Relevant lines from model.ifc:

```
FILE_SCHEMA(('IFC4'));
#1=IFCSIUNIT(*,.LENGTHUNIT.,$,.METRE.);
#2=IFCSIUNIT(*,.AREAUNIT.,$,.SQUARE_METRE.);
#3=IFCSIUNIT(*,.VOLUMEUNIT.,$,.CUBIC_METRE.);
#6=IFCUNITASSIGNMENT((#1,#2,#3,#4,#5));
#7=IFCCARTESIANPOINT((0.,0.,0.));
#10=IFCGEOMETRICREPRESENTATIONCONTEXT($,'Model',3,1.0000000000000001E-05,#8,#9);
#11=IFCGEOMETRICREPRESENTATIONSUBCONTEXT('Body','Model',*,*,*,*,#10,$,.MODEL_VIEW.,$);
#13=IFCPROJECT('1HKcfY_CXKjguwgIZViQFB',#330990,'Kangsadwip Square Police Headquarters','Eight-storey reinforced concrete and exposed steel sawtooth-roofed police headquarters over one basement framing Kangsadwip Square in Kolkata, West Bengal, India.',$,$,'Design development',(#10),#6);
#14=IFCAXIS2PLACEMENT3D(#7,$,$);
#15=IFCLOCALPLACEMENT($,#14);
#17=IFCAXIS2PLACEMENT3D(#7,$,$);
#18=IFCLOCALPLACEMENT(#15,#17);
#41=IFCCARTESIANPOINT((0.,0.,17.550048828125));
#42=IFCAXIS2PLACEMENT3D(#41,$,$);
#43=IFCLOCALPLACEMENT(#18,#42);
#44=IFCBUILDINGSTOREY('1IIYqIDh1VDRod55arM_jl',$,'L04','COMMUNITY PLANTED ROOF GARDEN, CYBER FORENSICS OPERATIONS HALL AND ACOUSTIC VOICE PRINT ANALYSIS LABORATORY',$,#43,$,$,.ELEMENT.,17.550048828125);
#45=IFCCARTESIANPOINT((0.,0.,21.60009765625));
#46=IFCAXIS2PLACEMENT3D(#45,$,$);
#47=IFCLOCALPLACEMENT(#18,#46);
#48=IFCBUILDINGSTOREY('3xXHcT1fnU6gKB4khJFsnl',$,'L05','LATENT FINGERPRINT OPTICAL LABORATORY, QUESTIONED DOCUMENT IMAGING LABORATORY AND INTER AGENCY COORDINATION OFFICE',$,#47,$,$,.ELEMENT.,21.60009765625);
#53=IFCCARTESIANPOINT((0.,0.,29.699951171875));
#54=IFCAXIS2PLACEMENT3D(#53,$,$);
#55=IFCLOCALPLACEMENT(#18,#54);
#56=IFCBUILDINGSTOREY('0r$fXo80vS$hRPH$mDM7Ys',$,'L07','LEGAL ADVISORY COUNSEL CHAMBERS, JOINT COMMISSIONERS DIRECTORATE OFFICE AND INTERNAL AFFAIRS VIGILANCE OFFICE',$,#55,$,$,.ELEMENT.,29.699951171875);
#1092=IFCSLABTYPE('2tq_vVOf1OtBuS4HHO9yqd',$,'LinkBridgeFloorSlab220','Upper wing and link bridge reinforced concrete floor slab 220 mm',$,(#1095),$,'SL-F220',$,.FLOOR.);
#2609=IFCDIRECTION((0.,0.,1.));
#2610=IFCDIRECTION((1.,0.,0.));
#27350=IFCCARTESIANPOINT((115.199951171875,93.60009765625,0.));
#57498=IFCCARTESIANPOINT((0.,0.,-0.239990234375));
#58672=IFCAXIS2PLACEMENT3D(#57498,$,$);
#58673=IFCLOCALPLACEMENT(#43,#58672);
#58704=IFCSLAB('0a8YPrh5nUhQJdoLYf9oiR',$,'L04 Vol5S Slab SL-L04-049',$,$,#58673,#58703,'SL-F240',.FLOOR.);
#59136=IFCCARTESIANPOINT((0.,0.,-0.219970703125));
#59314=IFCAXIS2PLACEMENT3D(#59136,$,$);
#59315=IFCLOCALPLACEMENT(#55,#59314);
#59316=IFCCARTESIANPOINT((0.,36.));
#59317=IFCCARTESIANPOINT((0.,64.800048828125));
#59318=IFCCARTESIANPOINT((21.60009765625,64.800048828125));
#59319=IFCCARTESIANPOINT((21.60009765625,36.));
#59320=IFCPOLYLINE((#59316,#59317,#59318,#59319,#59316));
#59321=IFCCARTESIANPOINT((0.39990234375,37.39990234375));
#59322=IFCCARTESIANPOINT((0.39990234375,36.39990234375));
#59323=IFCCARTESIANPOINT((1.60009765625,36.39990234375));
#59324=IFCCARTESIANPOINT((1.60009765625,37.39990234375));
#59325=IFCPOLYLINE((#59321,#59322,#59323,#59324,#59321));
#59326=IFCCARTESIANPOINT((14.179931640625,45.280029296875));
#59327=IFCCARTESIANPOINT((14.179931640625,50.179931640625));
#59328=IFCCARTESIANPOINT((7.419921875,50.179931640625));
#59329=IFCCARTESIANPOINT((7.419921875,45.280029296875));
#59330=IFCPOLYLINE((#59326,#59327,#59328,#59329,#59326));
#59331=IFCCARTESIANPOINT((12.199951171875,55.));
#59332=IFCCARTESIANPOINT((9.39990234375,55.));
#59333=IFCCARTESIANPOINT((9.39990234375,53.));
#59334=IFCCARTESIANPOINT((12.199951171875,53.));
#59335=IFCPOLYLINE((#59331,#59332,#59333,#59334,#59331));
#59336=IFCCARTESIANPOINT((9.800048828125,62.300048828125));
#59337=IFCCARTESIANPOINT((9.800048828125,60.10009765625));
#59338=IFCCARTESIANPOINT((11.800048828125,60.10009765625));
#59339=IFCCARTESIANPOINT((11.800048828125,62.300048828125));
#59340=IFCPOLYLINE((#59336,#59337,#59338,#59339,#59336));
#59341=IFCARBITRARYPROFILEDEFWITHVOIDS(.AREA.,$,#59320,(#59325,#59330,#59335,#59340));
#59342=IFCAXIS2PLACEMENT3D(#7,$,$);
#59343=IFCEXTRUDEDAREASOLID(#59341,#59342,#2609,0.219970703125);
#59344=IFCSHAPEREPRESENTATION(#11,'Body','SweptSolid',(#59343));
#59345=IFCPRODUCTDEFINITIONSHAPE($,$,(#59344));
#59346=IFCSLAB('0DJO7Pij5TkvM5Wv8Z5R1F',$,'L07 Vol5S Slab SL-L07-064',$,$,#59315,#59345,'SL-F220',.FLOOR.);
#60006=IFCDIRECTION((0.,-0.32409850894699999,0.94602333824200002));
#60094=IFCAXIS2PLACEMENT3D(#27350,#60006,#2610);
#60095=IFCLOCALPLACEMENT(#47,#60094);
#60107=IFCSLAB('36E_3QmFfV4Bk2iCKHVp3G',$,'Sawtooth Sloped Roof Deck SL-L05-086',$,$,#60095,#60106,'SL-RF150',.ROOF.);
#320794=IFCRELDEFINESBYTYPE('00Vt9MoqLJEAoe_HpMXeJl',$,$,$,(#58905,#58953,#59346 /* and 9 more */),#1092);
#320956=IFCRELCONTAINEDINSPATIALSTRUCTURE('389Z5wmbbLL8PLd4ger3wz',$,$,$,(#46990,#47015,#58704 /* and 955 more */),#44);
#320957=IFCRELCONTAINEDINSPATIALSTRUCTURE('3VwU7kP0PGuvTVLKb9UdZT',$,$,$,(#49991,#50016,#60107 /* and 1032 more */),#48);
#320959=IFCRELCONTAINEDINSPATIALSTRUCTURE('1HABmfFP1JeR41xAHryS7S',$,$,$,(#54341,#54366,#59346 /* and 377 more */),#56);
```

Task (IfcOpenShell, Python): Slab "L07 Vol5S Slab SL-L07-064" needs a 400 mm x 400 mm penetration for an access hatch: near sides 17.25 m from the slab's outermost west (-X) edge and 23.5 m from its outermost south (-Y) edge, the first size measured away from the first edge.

```python
import numpy as np
import ifcopenshell
import ifcopenshell.api.feature
import ifcopenshell.api.geometry
import ifcopenshell.api.root
import ifcopenshell.geom
import ifcopenshell.util.placement
import ifcopenshell.util.representation
import ifcopenshell.util.shape
import ifcopenshell.util.unit

model = ifcopenshell.open("model.ifc")
unit_scale = ifcopenshell.util.unit.calculate_unit_scale(model)
settings = ifcopenshell.geom.settings()


def volume(element):
    """Net volume in cubic metres, openings subtracted."""
    shape = ifcopenshell.geom.create_shape(settings, element)
    return ifcopenshell.util.shape.get_volume(shape.geometry)


slab = model.by_guid("0DJO7Pij5TkvM5Wv8Z5R1F")
before = volume(slab)

# Extent in the slab's own axes, in metres. The edges named are its -X and -Y sides.
slab_shape = ifcopenshell.geom.create_shape(settings, slab)
vertices = ifcopenshell.util.shape.get_vertices(slab_shape.geometry)
x_min, y_min, bottom = vertices.min(axis=0)
top = vertices[:, 2].max()

opening = ifcopenshell.api.root.create_entity(model, ifc_class="IfcOpeningElement", name="Access hatch opening", predefined_type="OPENING")
context = ifcopenshell.util.representation.get_context(model, "Model", "Body", "MODEL_VIEW")
width, depth = 0.4, 0.4
outline = [(0.0, 0.0), (width, 0.0), (width, depth), (0.0, depth), (0.0, 0.0)]
# Overshoot both faces by 50 mm so the cut is clean.
shape = ifcopenshell.api.geometry.add_slab_representation(
    model, context=context, depth=top - bottom + 0.1, polyline=outline
)
ifcopenshell.api.geometry.assign_representation(model, product=opening, representation=shape)

matrix = ifcopenshell.util.placement.get_local_placement(slab.ObjectPlacement)
matrix[:, 3] = matrix @ np.append(np.array([x_min + 17.25, y_min + 23.5, bottom - 0.05]) / unit_scale, 1.0)
ifcopenshell.api.geometry.edit_object_placement(model, product=opening, matrix=matrix, is_si=False)
ifcopenshell.api.feature.add_feature(model, feature=opening, element=slab)

after = volume(slab)

print(f"slab volume {before:.3f} -> {after:.3f} m3")

model.write("model_rev.ifc")
```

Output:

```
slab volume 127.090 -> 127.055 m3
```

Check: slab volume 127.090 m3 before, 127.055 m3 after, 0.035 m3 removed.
